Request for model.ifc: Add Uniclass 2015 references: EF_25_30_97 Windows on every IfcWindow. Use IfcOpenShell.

First a look at what the model holds.

```python
import ifcopenshell

model = ifcopenshell.open("model.ifc")
print(model.schema)
print("classifications:", [c.Name for c in model.by_type("IfcClassification")])
for ifc_class in ("IfcDoor", "IfcRoof", "IfcStair", "IfcWall", "IfcWindow"):
    print(ifc_class, len(model.by_type(ifc_class)))
```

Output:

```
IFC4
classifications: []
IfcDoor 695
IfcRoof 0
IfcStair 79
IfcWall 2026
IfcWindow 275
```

```python
import ifcopenshell
import ifcopenshell.api.classification

model = ifcopenshell.open("model.ifc")

system = ifcopenshell.api.classification.add_classification(model, classification="Uniclass 2015")

codes = {
    "IfcWindow": ("EF_25_30_97", "Windows"),
}
for ifc_class, (code, name) in codes.items():
    products = model.by_type(ifc_class)
    ifcopenshell.api.classification.add_reference(
        model, products=products, classification=system, identification=code, name=name
    )
    print(code, len(products))

model.write("model_v2.ifc")
```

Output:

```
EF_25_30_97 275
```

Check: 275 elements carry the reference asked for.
